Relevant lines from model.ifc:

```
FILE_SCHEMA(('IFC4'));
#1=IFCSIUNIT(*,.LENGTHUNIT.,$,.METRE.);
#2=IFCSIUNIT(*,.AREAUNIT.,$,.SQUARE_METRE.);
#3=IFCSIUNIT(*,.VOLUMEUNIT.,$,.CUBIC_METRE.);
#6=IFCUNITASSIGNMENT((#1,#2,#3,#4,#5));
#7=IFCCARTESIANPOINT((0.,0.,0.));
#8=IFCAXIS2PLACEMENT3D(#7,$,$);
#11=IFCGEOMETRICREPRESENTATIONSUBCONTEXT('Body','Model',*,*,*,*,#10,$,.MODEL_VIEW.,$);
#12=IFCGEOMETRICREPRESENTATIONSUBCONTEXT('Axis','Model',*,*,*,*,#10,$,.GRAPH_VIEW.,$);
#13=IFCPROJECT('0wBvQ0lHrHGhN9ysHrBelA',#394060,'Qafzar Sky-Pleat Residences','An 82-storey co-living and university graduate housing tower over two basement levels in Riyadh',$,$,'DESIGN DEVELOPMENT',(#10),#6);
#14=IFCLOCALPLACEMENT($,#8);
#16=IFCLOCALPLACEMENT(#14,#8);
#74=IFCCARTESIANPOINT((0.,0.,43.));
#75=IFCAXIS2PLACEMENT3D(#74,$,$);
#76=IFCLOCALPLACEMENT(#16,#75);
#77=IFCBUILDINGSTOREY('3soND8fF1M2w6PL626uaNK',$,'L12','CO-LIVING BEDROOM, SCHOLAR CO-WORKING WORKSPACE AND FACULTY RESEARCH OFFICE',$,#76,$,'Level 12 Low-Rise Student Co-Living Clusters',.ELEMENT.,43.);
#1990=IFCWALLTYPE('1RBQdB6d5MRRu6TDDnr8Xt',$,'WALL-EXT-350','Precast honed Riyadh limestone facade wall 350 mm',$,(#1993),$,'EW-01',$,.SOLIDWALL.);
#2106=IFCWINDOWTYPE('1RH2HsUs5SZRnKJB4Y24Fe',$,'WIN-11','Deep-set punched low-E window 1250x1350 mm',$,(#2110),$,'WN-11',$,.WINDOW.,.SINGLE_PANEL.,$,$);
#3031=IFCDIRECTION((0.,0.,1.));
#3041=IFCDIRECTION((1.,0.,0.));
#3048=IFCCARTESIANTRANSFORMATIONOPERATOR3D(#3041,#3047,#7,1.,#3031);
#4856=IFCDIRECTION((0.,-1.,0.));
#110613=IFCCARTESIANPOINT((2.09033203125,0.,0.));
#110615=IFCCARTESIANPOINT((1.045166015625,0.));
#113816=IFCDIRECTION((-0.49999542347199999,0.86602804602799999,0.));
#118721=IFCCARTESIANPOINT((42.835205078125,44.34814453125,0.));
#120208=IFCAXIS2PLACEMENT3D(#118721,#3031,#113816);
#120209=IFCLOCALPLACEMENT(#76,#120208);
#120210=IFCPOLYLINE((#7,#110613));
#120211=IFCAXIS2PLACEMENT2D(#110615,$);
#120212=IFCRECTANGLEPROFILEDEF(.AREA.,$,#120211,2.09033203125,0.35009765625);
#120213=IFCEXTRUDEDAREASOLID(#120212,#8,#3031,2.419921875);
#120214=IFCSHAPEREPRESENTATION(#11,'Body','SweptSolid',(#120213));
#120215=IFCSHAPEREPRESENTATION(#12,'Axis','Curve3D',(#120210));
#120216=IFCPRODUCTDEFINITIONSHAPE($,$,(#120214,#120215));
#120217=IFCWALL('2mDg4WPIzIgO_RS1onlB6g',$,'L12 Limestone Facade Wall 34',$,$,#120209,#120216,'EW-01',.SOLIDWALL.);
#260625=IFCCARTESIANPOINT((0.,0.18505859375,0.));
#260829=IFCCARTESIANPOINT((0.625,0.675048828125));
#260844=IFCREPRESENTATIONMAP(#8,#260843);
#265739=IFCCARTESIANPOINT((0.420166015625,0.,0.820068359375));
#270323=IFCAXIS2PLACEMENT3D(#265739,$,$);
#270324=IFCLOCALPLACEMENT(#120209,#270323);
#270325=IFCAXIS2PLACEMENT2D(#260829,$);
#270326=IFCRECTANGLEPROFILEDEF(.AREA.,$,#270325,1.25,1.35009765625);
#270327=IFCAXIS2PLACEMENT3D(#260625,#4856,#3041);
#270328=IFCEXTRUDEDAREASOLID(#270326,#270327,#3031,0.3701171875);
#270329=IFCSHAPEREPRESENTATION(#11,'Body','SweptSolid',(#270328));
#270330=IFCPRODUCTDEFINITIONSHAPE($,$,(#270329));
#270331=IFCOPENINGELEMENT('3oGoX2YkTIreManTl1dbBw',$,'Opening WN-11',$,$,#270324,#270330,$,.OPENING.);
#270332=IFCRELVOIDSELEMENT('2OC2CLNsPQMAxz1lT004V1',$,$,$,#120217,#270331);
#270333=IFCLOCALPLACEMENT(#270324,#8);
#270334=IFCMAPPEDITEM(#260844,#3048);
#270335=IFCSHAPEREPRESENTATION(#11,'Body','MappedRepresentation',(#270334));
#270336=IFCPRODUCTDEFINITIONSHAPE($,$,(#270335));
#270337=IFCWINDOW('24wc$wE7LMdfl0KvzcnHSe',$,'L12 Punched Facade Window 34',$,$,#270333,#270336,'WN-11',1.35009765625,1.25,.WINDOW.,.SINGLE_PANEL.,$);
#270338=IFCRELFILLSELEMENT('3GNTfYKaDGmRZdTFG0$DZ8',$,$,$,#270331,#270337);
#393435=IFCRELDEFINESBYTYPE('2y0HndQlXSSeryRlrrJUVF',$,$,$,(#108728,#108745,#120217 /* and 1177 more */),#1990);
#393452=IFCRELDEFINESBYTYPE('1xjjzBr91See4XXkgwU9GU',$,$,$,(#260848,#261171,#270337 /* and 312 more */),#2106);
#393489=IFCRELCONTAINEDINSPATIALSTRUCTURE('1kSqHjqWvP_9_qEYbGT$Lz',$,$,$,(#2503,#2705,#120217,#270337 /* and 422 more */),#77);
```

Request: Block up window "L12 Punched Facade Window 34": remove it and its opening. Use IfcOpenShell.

```python
import ifcopenshell
import ifcopenshell.api.feature
import ifcopenshell.api.root
import ifcopenshell.geom
import ifcopenshell.util.shape

model = ifcopenshell.open("model.ifc")
settings = ifcopenshell.geom.settings()


def volume(element):
    """Net volume in cubic metres, openings subtracted."""
    shape = ifcopenshell.geom.create_shape(settings, element)
    return ifcopenshell.util.shape.get_volume(shape.geometry)


window = model.by_id(270337)
opening = window.FillsVoids[0].RelatingOpeningElement
wall = opening.VoidsElements[0].RelatingBuildingElement
before = volume(wall)

ifcopenshell.api.root.remove_product(model, product=window)
ifcopenshell.api.feature.remove_feature(model, feature=opening)

after = volume(wall)

print(f"wall volume {before:.3f} -> {after:.3f} m3")

model.write("model_edited.ifc")
```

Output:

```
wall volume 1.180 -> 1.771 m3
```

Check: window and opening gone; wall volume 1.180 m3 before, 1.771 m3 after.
